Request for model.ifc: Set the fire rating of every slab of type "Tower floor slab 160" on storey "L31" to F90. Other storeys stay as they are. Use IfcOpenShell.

First a look at what the model holds.

```python
import ifcopenshell
import ifcopenshell.util.element

model = ifcopenshell.open("model.ifc")
print(model.schema)
storey = next(s for s in model.by_type("IfcBuildingStorey") if s.Name == "L31")
slabs = [e for e in ifcopenshell.util.element.get_decomposition(storey) if e.is_a("IfcSlab")]
seen = {}
for e in slabs:
    element_type = ifcopenshell.util.element.get_type(e)
    key = (element_type.Name if element_type != e and element_type else None, ifcopenshell.util.element.get_pset(e, "Pset_SlabCommon", "FireRating"))
    seen[key] = seen.get(key, 0) + 1
for (name, value), count in sorted(seen.items(), key=str):
    print(count, "x", name, "|", value)
```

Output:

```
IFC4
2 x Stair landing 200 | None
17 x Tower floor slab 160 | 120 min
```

```python
import ifcopenshell
import ifcopenshell.api.pset
import ifcopenshell.util.element

model = ifcopenshell.open("model.ifc")

storey = next(s for s in model.by_type("IfcBuildingStorey") if s.Name == "L31")
slabs = [e for e in ifcopenshell.util.element.get_decomposition(storey) if e.is_a("IfcSlab")]

count = 0
for e in slabs:
    element_type = ifcopenshell.util.element.get_type(e)
    if element_type in (None, e) or element_type.Name != "Tower floor slab 160":
        continue
    found = ifcopenshell.util.element.get_pset(e, "Pset_SlabCommon", should_inherit=False)
    if found:
        pset = model.by_id(found["id"])
        if len(ifcopenshell.util.element.get_elements_by_pset(pset)) > 1:
            pset = ifcopenshell.api.pset.unshare_pset(model, products=[e], pset=pset)[0]
    else:
        pset = ifcopenshell.api.pset.add_pset(model, product=e, name="Pset_SlabCommon")
    ifcopenshell.api.pset.edit_pset(model, pset=pset, properties={"FireRating": "F90"})
    count += 1

print(count, "slabs updated")

model.write("model-out.ifc")
```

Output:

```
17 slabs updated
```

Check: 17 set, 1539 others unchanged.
